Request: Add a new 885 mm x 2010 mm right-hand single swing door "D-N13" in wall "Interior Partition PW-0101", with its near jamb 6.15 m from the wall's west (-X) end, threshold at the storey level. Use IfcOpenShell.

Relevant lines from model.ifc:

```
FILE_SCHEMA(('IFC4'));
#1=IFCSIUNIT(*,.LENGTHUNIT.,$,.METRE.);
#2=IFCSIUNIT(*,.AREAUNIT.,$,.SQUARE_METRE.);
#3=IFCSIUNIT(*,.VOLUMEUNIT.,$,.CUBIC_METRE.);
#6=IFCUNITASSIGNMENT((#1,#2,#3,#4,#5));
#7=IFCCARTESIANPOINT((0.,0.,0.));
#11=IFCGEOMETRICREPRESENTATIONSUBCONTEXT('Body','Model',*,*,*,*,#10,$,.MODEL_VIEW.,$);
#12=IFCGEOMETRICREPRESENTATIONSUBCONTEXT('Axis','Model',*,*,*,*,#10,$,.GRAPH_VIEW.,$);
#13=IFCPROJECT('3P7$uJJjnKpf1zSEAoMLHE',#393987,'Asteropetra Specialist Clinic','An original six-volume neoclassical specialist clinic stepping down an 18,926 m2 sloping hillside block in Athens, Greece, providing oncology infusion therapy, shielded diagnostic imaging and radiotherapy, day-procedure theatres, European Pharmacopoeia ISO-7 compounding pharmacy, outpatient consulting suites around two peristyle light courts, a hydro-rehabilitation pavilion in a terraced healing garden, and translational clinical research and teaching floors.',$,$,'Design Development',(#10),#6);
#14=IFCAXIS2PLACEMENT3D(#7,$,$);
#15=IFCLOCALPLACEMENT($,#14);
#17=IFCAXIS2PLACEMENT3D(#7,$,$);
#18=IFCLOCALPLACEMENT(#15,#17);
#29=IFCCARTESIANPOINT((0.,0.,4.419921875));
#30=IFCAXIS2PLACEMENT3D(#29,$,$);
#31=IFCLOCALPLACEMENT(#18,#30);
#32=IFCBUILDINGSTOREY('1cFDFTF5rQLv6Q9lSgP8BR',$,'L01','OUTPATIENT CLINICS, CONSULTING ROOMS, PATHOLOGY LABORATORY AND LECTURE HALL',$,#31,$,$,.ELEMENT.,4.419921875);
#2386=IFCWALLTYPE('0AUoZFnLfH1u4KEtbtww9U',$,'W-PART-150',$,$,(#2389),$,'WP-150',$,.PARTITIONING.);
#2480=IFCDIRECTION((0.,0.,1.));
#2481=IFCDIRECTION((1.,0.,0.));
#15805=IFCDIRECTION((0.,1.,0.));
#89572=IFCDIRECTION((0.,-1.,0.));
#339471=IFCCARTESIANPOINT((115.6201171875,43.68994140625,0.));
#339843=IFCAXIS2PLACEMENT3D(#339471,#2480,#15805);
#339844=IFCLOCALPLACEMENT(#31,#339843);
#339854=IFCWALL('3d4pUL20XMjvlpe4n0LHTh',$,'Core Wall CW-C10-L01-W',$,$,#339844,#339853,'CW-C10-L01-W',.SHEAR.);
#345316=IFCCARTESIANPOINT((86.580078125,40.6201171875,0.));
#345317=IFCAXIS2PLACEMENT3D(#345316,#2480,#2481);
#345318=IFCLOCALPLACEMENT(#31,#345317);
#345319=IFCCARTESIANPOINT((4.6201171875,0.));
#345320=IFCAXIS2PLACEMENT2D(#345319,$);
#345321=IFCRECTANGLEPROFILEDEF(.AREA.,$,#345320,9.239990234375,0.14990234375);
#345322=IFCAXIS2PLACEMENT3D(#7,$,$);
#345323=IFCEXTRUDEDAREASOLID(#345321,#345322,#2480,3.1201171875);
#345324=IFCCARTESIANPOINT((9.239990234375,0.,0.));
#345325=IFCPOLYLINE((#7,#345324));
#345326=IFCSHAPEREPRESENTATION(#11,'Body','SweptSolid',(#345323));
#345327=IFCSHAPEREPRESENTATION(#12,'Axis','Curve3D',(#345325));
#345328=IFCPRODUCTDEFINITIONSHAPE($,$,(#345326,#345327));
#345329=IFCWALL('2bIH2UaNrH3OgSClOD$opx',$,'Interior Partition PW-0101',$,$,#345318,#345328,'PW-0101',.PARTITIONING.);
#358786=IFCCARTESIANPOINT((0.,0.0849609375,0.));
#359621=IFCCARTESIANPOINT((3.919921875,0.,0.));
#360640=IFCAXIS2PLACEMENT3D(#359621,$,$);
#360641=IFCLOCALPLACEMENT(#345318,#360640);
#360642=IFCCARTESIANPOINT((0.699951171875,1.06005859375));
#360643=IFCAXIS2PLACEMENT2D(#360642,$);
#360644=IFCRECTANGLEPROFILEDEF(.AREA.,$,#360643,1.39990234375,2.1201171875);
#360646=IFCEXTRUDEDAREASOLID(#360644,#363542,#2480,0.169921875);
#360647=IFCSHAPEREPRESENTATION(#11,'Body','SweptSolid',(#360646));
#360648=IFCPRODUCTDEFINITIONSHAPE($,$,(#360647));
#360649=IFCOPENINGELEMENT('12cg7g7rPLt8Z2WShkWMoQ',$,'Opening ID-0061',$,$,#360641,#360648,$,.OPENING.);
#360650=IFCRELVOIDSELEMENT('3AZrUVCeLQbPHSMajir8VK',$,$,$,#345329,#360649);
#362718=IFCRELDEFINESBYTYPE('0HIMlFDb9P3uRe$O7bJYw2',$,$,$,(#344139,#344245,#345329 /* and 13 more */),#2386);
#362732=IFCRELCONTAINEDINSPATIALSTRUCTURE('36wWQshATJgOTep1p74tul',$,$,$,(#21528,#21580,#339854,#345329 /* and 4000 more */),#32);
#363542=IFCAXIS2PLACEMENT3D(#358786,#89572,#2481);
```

```python
import numpy as np
import ifcopenshell
import ifcopenshell.api.feature
import ifcopenshell.api.geometry
import ifcopenshell.api.root
import ifcopenshell.api.spatial
import ifcopenshell.geom
import ifcopenshell.util.element
import ifcopenshell.util.placement
import ifcopenshell.util.representation
import ifcopenshell.util.shape
import ifcopenshell.util.unit

model = ifcopenshell.open("model.ifc")
unit_scale = ifcopenshell.util.unit.calculate_unit_scale(model)
settings = ifcopenshell.geom.settings()


def volume(element):
    """Net volume in cubic metres, openings subtracted."""
    shape = ifcopenshell.geom.create_shape(settings, element)
    return ifcopenshell.util.shape.get_volume(shape.geometry)


wall = model.by_guid("2bIH2UaNrH3OgSClOD$opx")
storey = ifcopenshell.util.element.get_container(wall, ifc_class="IfcBuildingStorey")
context = ifcopenshell.util.representation.get_context(model, "Model", "Body", "MODEL_VIEW")
before = volume(wall)

width, height, from_end, sill = 0.885, 2.01, 6.15, 0.0  # metres

# The wall runs along its own X axis, and the end named is its -X end.
wall_shape = ifcopenshell.geom.create_shape(settings, wall)
x, y, z = ifcopenshell.util.shape.get_vertices(wall_shape.geometry).T
start = x.min() + from_end
face, thickness = float(y.min()), float(y.max() - y.min())
wall_matrix = ifcopenshell.util.placement.get_local_placement(wall.ObjectPlacement)
level = ifcopenshell.util.placement.get_local_placement(storey.ObjectPlacement)[2, 3]


def in_wall(x, y):
    """Placement at x, y metres in the wall's axes, at sill height."""
    matrix = wall_matrix.copy()
    matrix[:, 3] = wall_matrix @ np.array([x / unit_scale, y / unit_scale, 0.0, 1.0])
    matrix[2, 3] = level + sill / unit_scale
    return matrix


# Opening: a box that overshoots both wall faces by 50 mm.
opening = ifcopenshell.api.root.create_entity(model, ifc_class="IfcOpeningElement", predefined_type="OPENING")
box = ifcopenshell.api.geometry.add_wall_representation(
    model, context=context, length=width, height=height, thickness=thickness + 0.1
)
ifcopenshell.api.geometry.assign_representation(model, product=opening, representation=box)
ifcopenshell.api.geometry.edit_object_placement(model, product=opening, matrix=in_wall(start, face - 0.05), is_si=False)
ifcopenshell.api.feature.add_feature(model, feature=opening, element=wall)

door = ifcopenshell.api.root.create_entity(model, ifc_class="IfcDoor", name="D-N13", predefined_type="DOOR")
door.OverallWidth, door.OverallHeight = width / unit_scale, height / unit_scale
door.OperationType = "SINGLE_SWING_RIGHT"
body = ifcopenshell.api.geometry.add_door_representation(
    model,
    context=context,
    overall_width=door.OverallWidth,
    overall_height=door.OverallHeight,
    operation_type="SINGLE_SWING_RIGHT",
    lining_properties={"LiningDepth": thickness / unit_scale, "ThresholdDepth": thickness / unit_scale},
)
ifcopenshell.api.geometry.assign_representation(model, product=door, representation=body)
ifcopenshell.api.spatial.assign_container(model, products=[door], relating_structure=storey)
ifcopenshell.api.feature.add_filling(model, opening=opening, element=door)

# The lining spans the wall, so the door starts at the wall face.
ifcopenshell.api.geometry.edit_object_placement(model, product=door, matrix=in_wall(start, face), is_si=False)

after = volume(wall)

print(f"wall volume {before:.3f} -> {after:.3f} m3")

model.write("model_v2.ifc")
```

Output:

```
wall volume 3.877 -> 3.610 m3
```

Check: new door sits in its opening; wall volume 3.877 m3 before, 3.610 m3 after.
